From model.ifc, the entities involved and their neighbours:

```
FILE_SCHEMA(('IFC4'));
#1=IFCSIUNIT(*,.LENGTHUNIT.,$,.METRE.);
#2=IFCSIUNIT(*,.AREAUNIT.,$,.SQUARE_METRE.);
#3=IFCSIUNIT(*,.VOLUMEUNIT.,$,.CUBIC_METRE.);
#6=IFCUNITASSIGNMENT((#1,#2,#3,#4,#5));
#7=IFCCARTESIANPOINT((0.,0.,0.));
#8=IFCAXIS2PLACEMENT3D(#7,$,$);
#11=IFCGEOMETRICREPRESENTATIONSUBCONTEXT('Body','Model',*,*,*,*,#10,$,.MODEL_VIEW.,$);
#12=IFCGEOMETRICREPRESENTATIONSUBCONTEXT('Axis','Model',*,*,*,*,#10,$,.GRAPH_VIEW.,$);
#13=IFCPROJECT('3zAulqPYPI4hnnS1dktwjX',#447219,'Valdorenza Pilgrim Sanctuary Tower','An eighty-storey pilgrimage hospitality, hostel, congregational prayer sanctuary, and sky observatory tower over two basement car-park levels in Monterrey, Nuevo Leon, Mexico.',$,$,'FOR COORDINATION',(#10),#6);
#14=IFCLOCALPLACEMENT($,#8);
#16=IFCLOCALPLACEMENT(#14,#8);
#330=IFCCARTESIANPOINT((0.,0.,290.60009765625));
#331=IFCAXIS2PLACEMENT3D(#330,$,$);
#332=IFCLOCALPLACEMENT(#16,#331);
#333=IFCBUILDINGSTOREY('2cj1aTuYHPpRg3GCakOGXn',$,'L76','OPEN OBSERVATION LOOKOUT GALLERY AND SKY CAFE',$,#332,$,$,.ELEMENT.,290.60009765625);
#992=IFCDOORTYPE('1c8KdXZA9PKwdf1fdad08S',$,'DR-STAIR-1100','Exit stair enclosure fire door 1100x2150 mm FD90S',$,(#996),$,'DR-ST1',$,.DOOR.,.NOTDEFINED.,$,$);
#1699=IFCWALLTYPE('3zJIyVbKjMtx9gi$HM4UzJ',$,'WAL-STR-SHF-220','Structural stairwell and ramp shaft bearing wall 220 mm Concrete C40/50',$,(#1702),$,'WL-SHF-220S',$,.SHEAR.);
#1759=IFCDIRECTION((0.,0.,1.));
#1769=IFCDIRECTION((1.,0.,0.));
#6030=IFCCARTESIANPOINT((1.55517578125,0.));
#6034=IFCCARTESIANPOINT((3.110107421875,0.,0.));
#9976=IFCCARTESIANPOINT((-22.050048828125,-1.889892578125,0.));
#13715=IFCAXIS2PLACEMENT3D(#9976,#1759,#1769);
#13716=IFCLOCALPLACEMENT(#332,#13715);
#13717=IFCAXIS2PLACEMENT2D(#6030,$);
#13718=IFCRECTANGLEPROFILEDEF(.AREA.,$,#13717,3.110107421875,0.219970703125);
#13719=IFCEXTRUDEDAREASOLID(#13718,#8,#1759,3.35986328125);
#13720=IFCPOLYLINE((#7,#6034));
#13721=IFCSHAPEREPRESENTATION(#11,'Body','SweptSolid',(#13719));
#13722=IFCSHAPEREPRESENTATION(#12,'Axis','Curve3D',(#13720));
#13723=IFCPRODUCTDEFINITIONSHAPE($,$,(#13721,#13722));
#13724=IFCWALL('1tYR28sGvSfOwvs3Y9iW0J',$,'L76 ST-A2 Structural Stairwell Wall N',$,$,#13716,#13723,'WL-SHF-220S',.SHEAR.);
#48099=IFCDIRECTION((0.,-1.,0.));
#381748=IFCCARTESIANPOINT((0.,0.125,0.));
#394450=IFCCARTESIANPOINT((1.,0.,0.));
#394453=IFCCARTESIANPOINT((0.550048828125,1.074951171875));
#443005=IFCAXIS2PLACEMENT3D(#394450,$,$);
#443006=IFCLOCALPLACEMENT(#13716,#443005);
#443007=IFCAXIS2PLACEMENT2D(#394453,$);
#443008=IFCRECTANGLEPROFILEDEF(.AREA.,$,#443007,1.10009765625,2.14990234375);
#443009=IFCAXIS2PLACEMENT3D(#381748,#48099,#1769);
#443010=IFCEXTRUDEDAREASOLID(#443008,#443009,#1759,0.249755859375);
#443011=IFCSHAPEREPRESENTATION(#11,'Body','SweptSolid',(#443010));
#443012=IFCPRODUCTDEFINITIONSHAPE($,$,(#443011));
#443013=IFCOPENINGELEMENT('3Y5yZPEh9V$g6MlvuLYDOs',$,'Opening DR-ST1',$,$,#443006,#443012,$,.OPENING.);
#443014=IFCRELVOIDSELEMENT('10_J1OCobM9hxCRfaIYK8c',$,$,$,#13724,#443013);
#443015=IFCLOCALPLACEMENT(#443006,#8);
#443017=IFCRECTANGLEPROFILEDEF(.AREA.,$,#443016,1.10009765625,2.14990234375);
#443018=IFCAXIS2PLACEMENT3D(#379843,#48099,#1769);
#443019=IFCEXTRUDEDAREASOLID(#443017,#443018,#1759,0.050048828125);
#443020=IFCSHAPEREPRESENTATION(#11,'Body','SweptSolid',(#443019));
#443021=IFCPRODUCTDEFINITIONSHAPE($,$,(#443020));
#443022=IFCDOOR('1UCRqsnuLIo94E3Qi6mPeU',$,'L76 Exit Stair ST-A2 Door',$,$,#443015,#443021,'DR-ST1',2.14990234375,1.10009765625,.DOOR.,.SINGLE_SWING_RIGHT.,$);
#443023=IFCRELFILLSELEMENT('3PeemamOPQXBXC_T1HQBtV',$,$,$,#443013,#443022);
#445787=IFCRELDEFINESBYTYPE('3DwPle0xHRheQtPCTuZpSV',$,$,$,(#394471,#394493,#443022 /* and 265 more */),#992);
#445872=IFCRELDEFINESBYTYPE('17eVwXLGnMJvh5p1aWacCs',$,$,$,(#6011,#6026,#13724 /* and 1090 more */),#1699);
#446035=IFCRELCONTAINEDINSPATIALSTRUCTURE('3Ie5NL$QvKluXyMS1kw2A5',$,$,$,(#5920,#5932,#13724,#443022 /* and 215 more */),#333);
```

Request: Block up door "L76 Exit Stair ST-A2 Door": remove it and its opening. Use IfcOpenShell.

```python
import ifcopenshell
import ifcopenshell.api.feature
import ifcopenshell.api.root
import ifcopenshell.geom
import ifcopenshell.util.shape

model = ifcopenshell.open("model.ifc")
settings = ifcopenshell.geom.settings()


def volume(element):
    """Net volume in cubic metres, openings subtracted."""
    shape = ifcopenshell.geom.create_shape(settings, element)
    return ifcopenshell.util.shape.get_volume(shape.geometry)


door = model.by_guid("1UCRqsnuLIo94E3Qi6mPeU")
opening = door.FillsVoids[0].RelatingOpeningElement
wall = opening.VoidsElements[0].RelatingBuildingElement
before = volume(wall)

ifcopenshell.api.root.remove_product(model, product=door)
ifcopenshell.api.feature.remove_feature(model, feature=opening)

after = volume(wall)

print(f"wall volume {before:.3f} -> {after:.3f} m3")

model.write("model_edited.ifc")
```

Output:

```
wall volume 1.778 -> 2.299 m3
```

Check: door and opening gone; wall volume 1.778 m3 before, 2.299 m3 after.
